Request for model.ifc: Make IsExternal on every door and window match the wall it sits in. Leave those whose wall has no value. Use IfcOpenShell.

First a look at what the model holds.

```python
import ifcopenshell
import ifcopenshell.util.element

model = ifcopenshell.open("model.ifc")
print(model.schema)
seen = {}
for e in model.by_type("IfcDoor") + model.by_type("IfcWindow"):
    if not e.FillsVoids:
        continue
    host = e.FillsVoids[0].RelatingOpeningElement.VoidsElements[0].RelatingBuildingElement
    own = ifcopenshell.util.element.get_pset(e, f"Pset_{e.is_a()[3:].removesuffix('StandardCase')}Common", "IsExternal")
    wall = ifcopenshell.util.element.get_pset(host, "Pset_WallCommon", "IsExternal")
    seen[e.is_a(), own, wall] = seen.get((e.is_a(), own, wall), 0) + 1
for (cls, own, wall), count in sorted(seen.items(), key=str):
    print(count, cls, "IsExternal:", own, "| host wall:", wall)
```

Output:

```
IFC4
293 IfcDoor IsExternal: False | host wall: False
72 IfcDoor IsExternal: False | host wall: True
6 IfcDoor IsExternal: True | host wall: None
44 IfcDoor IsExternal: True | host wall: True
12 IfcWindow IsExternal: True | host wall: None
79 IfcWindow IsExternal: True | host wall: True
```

```python
import ifcopenshell
import ifcopenshell.api.pset
import ifcopenshell.util.element

model = ifcopenshell.open("model.ifc")

count = 0
for ifc_class, pset_name in (("IfcDoor", "Pset_DoorCommon"), ("IfcWindow", "Pset_WindowCommon")):
    for e in model.by_type(ifc_class):
        if not e.FillsVoids:
            continue
        host = e.FillsVoids[0].RelatingOpeningElement.VoidsElements[0].RelatingBuildingElement
        external = ifcopenshell.util.element.get_pset(host, "Pset_WallCommon", "IsExternal")
        if external is None or ifcopenshell.util.element.get_pset(e, pset_name, "IsExternal") == external:
            continue
        pset = ifcopenshell.api.pset.add_pset(model, product=e, name=pset_name)
        ifcopenshell.api.pset.edit_pset(model, pset=pset, properties={"IsExternal": external})
        count += 1

print(count, "updated")

model.write("model_v2.ifc")
```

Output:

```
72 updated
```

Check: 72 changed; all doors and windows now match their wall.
